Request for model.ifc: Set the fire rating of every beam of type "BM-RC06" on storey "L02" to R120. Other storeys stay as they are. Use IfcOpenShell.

First a look at what the model holds.

```python
import ifcopenshell
import ifcopenshell.util.element

model = ifcopenshell.open("model.ifc")
print(model.schema)
storey = next(s for s in model.by_type("IfcBuildingStorey") if s.Name == "L02")
beams = [e for e in ifcopenshell.util.element.get_decomposition(storey) if e.is_a("IfcBeam")]
seen = {}
for e in beams:
    element_type = ifcopenshell.util.element.get_type(e)
    key = (element_type.Name if element_type != e and element_type else None, ifcopenshell.util.element.get_pset(e, "Pset_BeamCommon", "FireRating"))
    seen[key] = seen.get(key, 0) + 1
for (name, value), count in sorted(seen.items(), key=str):
    print(count, "x", name, "|", value)
```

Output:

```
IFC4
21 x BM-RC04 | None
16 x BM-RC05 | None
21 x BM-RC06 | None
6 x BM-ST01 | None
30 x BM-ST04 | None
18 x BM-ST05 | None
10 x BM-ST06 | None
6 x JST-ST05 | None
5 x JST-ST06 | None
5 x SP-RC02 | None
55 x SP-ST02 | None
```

```python
import ifcopenshell
import ifcopenshell.api.pset
import ifcopenshell.util.element

model = ifcopenshell.open("model.ifc")

storey = next(s for s in model.by_type("IfcBuildingStorey") if s.Name == "L02")
beams = [e for e in ifcopenshell.util.element.get_decomposition(storey) if e.is_a("IfcBeam")]

count = 0
for e in beams:
    element_type = ifcopenshell.util.element.get_type(e)
    if element_type in (None, e) or element_type.Name != "BM-RC06":
        continue
    # add_pset returns the element's existing set when there is one.
    pset = ifcopenshell.api.pset.add_pset(model, product=e, name="Pset_BeamCommon")
    ifcopenshell.api.pset.edit_pset(model, pset=pset, properties={"FireRating": "R120"})
    count += 1

print(count, "beams updated")

model.write("model_edited.ifc")
```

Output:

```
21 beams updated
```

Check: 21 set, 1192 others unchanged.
